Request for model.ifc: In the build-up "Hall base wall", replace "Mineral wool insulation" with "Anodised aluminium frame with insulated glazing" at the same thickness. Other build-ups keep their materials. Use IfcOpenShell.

First a look at what the model holds.

```python
import ifcopenshell
import ifcopenshell.util.element

model = ifcopenshell.open("model.ifc")
print(model.schema)
for layer_set in model.by_type("IfcMaterialLayerSet"):
    if layer_set.LayerSetName == "Hall base wall":
        for layer in layer_set.MaterialLayers:
            print(layer.id(), layer.Material and layer.Material.Name, layer.LayerThickness, sep=" | ")
        print(len(ifcopenshell.util.element.get_elements_by_material(model, layer_set)), "elements and types use it")
print(sorted(m.Name for m in model.by_type("IfcMaterial") if m.Name)[:60])
```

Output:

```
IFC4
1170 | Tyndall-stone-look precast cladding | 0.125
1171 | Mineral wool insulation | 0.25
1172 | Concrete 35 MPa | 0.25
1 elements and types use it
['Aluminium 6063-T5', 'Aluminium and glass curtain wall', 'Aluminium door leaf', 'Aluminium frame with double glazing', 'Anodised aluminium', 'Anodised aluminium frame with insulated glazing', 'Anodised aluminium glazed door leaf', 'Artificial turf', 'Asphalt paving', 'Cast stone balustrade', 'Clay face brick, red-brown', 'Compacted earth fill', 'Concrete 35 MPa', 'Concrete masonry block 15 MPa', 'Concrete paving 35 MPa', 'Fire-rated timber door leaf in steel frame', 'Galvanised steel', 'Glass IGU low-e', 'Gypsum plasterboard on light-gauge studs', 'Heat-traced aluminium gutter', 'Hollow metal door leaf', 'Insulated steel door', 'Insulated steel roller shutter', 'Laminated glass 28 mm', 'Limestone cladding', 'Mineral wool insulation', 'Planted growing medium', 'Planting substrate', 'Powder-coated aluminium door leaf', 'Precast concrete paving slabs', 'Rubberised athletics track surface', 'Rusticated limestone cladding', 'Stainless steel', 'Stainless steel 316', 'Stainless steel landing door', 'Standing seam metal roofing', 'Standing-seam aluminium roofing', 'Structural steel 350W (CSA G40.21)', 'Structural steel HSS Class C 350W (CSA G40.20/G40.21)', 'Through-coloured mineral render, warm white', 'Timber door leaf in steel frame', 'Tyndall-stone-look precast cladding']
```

```python
import ifcopenshell
import ifcopenshell.api.material

model = ifcopenshell.open("model.ifc")

layer_set = next(s for s in model.by_type("IfcMaterialLayerSet") if s.LayerSetName == "Hall base wall")
layer = next(l for l in layer_set.MaterialLayers if l.Material and l.Material.Name == "Mineral wool insulation")
material = next(m for m in model.by_type("IfcMaterial") if m.Name == "Anodised aluminium frame with insulated glazing")

# Point this one layer at the other material; renaming the old one would change it everywhere.
ifcopenshell.api.material.edit_layer(model, layer=layer, attributes={"Name": material.Name}, material=material)

print([l.Material.Name if l.Material else None for l in layer_set.MaterialLayers])

model.write("model_v2.ifc")
```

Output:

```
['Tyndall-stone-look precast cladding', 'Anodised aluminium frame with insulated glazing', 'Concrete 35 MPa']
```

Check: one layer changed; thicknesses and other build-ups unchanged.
